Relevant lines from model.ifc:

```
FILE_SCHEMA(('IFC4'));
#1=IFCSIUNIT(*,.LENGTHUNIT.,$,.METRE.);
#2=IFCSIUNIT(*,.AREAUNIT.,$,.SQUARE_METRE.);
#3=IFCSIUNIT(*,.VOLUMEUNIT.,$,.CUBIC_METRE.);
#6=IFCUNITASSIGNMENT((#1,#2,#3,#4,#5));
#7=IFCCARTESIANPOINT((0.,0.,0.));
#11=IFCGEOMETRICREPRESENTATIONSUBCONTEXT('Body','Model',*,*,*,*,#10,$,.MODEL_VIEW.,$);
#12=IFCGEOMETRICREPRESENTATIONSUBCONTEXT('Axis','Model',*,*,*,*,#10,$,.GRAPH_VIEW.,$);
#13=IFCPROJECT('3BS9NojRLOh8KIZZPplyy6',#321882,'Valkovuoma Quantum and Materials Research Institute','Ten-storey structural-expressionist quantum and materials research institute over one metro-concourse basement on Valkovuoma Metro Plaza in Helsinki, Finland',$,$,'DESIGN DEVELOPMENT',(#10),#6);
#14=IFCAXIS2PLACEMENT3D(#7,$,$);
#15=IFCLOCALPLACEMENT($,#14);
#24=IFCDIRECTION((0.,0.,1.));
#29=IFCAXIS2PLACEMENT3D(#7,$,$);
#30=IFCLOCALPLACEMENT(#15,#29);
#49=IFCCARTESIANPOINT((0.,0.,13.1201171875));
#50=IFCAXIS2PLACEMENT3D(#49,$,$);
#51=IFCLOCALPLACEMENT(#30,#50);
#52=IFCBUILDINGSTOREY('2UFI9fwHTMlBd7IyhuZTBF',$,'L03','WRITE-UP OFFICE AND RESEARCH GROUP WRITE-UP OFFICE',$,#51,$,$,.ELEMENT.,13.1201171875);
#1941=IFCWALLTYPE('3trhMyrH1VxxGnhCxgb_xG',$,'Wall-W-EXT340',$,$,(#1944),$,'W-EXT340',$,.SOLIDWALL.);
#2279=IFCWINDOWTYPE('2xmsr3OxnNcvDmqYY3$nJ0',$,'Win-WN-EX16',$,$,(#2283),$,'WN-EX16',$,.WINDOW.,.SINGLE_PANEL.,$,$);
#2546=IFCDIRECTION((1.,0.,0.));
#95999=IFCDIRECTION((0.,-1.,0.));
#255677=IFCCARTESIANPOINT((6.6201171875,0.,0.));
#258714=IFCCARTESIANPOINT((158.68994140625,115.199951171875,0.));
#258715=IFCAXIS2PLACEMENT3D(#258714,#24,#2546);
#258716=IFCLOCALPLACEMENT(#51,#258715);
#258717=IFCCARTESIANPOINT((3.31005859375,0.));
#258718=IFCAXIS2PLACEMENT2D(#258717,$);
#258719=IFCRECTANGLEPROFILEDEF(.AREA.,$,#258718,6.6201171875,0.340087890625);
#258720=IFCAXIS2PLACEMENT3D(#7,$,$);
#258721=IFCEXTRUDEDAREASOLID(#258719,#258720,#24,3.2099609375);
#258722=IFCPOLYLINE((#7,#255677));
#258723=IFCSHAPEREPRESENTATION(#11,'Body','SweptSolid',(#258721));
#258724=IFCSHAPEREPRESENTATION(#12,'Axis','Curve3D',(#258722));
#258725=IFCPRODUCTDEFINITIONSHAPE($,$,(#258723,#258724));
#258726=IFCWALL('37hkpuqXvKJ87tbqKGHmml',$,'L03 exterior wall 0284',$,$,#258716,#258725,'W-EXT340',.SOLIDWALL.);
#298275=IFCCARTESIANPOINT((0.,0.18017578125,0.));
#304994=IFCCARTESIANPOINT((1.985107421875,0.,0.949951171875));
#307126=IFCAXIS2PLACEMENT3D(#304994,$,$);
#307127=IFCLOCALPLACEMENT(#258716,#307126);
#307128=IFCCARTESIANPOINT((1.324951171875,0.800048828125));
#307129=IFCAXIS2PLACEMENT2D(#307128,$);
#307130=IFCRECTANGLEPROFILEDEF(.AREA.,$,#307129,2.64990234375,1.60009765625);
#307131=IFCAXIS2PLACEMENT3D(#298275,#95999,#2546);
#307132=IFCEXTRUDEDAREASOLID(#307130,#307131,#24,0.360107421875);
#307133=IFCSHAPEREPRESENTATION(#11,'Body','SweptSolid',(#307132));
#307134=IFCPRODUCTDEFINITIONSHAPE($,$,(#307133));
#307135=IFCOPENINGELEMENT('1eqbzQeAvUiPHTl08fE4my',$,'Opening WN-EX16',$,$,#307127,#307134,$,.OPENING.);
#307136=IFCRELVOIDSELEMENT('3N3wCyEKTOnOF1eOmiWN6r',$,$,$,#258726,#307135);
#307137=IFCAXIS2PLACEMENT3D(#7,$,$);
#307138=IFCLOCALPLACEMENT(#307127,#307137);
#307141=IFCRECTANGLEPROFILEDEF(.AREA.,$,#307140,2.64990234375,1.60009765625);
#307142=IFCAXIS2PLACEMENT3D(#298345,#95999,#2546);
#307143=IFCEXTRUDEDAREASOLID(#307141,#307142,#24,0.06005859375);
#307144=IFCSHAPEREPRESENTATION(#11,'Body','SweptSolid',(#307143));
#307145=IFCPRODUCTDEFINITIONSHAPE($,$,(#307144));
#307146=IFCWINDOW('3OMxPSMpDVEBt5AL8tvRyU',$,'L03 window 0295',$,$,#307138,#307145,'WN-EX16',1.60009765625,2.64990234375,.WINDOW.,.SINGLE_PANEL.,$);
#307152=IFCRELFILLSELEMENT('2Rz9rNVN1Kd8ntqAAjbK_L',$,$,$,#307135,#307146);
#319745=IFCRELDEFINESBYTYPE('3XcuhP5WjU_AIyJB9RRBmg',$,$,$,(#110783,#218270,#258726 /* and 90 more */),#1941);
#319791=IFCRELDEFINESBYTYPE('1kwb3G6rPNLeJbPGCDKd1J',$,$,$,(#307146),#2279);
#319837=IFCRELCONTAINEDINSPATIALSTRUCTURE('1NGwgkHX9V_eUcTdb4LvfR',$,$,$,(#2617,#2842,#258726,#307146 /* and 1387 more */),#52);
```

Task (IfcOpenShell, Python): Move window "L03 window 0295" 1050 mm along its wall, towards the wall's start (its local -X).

```python
import ifcopenshell
import ifcopenshell.api.geometry
import ifcopenshell.util.placement

model = ifcopenshell.open("model.ifc")

window = model.by_guid("3OMxPSMpDVEBt5AL8tvRyU")
opening = window.FillsVoids[0].RelatingOpeningElement
wall = opening.VoidsElements[0].RelatingBuildingElement

wall_matrix = ifcopenshell.util.placement.get_local_placement(wall.ObjectPlacement)
shift = wall_matrix[:3, 0] * -1.05
before = ifcopenshell.util.placement.get_local_placement(window.ObjectPlacement)[:3, 3].copy()

# The window is placed relative to its opening, so it follows when the opening moves.
matrix = ifcopenshell.util.placement.get_local_placement(opening.ObjectPlacement)
matrix[:3, 3] += shift
ifcopenshell.api.geometry.edit_object_placement(
    model, product=opening, matrix=matrix, is_si=False, should_transform_children=True
)

after = ifcopenshell.util.placement.get_local_placement(window.ObjectPlacement)[:3, 3]
print("window moved by", (after - before).round(3) + 0.0)

model.write("model_edited.ifc")
```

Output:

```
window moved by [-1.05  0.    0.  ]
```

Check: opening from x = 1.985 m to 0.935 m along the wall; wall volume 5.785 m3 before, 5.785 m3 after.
